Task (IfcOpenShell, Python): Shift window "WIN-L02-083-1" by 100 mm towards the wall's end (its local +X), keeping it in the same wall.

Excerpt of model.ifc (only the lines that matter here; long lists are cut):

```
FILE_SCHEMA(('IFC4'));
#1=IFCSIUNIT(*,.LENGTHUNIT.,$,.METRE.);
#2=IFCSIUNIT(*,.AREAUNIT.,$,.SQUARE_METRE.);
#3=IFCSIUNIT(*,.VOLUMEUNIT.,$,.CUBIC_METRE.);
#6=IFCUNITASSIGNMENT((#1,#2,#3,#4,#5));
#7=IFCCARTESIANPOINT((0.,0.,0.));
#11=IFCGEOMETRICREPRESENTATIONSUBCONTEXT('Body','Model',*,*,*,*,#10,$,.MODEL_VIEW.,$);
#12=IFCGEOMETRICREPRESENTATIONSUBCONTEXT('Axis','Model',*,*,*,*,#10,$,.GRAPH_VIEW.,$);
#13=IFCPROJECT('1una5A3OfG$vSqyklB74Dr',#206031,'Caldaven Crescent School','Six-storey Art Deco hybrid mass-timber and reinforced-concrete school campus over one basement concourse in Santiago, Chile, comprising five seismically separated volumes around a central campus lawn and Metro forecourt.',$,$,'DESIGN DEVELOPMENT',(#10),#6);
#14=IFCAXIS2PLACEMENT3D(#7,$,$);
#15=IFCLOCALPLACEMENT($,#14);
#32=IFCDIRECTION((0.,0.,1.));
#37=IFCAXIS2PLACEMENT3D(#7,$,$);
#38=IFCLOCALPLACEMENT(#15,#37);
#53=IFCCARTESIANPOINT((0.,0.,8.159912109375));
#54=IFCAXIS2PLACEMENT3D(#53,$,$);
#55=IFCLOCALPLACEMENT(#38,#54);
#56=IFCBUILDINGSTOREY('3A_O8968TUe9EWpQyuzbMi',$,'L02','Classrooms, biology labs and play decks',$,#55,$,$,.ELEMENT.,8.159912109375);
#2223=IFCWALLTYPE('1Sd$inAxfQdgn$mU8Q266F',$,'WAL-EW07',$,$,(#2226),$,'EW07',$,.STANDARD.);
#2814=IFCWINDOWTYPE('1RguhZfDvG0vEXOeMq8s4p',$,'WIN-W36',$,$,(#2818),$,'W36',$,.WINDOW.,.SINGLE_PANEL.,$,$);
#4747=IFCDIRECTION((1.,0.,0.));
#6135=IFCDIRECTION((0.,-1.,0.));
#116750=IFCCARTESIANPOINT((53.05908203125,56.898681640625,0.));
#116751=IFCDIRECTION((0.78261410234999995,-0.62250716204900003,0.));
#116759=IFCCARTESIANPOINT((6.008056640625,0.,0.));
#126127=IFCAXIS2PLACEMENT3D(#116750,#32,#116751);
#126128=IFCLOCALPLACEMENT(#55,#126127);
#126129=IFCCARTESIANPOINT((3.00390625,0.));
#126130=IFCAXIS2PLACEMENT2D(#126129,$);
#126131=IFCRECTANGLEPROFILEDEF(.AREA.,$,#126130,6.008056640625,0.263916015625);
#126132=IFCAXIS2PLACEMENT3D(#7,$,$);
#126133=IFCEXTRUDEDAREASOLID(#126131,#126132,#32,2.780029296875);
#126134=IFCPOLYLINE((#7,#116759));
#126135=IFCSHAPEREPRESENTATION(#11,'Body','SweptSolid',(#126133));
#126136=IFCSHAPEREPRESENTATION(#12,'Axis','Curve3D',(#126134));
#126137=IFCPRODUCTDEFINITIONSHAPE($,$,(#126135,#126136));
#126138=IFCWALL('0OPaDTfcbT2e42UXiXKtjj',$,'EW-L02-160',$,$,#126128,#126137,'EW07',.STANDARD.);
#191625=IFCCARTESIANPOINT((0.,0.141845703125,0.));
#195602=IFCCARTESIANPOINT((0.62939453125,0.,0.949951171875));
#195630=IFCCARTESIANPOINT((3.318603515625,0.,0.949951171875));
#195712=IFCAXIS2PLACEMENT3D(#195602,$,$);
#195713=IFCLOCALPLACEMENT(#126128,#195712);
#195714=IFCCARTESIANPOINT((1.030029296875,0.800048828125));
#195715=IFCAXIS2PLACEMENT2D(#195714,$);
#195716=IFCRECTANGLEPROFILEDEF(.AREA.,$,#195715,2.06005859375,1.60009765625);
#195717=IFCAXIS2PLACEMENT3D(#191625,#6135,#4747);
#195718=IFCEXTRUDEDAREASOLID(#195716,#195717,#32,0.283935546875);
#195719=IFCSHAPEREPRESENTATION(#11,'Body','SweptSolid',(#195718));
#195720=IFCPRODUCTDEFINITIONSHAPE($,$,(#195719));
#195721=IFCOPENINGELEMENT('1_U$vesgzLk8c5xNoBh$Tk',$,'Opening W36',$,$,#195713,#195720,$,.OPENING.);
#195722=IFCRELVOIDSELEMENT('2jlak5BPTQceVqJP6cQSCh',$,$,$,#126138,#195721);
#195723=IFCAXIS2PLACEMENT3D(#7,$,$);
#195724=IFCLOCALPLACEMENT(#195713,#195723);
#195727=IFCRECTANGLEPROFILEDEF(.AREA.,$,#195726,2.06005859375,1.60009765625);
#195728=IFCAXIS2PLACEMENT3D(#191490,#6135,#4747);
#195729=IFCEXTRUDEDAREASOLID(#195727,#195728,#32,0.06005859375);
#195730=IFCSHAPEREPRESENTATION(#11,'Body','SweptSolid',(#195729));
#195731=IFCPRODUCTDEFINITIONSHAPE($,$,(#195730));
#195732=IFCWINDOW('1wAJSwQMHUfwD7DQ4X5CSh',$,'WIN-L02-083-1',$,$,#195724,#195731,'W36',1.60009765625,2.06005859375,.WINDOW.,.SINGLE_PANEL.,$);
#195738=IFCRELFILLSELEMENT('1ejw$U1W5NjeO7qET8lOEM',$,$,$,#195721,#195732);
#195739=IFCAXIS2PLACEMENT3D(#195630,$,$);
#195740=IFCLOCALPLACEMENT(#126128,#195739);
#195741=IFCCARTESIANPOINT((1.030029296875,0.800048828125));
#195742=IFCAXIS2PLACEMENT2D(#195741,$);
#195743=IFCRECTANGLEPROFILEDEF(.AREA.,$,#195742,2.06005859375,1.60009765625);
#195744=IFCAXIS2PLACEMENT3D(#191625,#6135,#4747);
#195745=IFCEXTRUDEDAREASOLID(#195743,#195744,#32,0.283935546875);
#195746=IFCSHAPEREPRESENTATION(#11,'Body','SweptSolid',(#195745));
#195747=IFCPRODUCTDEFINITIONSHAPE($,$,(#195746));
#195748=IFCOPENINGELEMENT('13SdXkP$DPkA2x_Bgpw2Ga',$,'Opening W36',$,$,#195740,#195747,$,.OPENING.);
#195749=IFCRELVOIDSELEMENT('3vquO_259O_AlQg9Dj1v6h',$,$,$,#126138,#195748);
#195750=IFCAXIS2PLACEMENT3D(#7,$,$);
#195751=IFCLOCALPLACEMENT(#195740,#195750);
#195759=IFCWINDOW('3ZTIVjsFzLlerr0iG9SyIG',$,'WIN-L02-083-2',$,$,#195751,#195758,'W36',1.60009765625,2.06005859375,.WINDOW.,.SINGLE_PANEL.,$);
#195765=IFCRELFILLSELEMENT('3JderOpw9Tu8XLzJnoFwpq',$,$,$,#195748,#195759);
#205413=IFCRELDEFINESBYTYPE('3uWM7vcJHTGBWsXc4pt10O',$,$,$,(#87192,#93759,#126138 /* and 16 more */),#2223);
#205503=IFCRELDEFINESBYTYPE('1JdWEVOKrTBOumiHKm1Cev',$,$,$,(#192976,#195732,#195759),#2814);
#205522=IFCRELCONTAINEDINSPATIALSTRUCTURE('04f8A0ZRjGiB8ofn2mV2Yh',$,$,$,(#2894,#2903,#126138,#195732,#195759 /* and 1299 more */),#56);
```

```python
import ifcopenshell
import ifcopenshell.api.geometry
import ifcopenshell.util.placement

model = ifcopenshell.open("model.ifc")

window = model.by_guid("1wAJSwQMHUfwD7DQ4X5CSh")
opening = window.FillsVoids[0].RelatingOpeningElement
wall = opening.VoidsElements[0].RelatingBuildingElement

wall_matrix = ifcopenshell.util.placement.get_local_placement(wall.ObjectPlacement)
shift = wall_matrix[:3, 0] * 0.1
before = ifcopenshell.util.placement.get_local_placement(window.ObjectPlacement)[:3, 3].copy()

# The window is placed relative to its opening, so it follows when the opening moves.
matrix = ifcopenshell.util.placement.get_local_placement(opening.ObjectPlacement)
matrix[:3, 3] += shift
ifcopenshell.api.geometry.edit_object_placement(
    model, product=opening, matrix=matrix, is_si=False, should_transform_children=True
)

after = ifcopenshell.util.placement.get_local_placement(window.ObjectPlacement)[:3, 3]
print("window moved by", (after - before).round(3) + 0.0)

model.write("model-out.ifc")
```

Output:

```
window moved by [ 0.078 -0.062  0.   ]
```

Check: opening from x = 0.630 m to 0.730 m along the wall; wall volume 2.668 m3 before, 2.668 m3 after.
